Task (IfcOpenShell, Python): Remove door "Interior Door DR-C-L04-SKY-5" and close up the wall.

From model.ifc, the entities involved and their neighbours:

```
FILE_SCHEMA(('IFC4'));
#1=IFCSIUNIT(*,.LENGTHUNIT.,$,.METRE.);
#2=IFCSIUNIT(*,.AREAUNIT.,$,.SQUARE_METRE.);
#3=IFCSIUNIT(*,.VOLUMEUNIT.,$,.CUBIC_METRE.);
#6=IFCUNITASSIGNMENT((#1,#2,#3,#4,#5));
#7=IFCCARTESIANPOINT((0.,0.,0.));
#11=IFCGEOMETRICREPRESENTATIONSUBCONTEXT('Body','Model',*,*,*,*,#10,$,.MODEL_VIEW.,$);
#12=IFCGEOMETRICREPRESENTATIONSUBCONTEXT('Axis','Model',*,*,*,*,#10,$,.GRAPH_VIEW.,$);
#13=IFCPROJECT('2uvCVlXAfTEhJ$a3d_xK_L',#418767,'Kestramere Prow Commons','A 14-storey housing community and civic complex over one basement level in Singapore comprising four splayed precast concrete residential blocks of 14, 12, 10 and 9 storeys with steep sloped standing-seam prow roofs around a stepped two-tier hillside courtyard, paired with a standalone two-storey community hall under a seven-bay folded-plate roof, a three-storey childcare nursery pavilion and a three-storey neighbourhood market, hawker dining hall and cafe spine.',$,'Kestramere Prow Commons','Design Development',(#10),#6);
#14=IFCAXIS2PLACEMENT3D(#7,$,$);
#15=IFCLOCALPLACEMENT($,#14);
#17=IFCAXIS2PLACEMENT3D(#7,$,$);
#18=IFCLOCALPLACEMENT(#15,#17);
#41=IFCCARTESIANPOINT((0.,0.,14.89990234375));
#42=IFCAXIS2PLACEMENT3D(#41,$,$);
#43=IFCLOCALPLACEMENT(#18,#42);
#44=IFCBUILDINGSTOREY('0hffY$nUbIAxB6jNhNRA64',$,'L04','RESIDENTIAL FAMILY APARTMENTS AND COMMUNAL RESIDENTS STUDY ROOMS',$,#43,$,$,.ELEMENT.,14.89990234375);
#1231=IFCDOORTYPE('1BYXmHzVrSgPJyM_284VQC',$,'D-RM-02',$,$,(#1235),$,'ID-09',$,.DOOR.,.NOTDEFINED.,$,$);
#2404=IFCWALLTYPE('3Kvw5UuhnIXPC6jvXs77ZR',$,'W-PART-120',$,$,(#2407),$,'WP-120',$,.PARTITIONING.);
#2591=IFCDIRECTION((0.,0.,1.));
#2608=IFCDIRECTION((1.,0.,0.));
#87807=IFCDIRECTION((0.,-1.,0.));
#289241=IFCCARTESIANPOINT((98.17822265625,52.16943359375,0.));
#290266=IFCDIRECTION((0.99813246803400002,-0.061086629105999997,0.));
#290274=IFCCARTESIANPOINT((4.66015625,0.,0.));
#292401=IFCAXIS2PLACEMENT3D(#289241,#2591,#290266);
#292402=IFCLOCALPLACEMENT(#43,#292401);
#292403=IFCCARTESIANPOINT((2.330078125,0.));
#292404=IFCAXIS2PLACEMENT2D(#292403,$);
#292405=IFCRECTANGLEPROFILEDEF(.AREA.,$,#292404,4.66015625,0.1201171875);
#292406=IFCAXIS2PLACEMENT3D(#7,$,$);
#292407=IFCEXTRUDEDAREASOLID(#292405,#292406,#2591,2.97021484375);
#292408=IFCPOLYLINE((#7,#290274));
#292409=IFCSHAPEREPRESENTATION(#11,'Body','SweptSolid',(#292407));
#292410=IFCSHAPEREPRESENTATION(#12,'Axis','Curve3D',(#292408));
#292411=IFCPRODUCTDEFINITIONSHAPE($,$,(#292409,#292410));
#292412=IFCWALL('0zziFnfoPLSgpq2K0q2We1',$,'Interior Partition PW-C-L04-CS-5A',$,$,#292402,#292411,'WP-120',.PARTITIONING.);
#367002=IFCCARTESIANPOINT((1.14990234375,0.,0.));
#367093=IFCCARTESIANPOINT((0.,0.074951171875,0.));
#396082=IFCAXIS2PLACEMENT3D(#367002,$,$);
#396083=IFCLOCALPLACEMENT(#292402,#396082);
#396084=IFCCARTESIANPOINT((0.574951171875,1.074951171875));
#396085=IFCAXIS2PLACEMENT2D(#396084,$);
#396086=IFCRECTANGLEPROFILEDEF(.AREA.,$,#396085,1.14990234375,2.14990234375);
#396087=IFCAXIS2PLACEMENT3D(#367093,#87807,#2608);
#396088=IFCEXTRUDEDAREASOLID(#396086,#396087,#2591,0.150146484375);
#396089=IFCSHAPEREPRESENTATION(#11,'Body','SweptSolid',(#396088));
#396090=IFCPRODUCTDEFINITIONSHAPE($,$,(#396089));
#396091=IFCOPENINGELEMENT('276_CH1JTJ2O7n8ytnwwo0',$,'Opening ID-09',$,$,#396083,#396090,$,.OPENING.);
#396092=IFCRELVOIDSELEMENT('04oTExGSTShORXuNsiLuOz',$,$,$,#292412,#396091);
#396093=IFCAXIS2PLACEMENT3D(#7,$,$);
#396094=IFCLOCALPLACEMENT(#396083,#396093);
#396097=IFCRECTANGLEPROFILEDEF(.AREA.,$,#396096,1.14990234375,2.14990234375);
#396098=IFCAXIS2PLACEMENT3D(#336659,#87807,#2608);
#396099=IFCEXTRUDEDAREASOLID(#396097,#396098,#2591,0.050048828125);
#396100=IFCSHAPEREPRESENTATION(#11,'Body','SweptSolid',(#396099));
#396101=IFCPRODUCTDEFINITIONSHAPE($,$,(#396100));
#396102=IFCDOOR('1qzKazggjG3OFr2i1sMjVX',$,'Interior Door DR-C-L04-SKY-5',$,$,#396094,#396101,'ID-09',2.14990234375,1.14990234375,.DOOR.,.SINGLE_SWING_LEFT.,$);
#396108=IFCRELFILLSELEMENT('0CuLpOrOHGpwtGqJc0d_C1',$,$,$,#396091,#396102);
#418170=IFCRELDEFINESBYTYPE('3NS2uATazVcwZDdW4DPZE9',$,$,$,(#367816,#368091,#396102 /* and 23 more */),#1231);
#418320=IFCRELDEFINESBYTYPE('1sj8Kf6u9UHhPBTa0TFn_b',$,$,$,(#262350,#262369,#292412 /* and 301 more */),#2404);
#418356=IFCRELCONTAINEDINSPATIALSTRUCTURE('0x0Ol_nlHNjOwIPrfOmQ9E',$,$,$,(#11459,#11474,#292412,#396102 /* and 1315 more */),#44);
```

```python
import ifcopenshell
import ifcopenshell.api.feature
import ifcopenshell.api.root
import ifcopenshell.geom
import ifcopenshell.util.shape

model = ifcopenshell.open("model.ifc")
settings = ifcopenshell.geom.settings()


def volume(element):
    """Net volume in cubic metres, openings subtracted."""
    shape = ifcopenshell.geom.create_shape(settings, element)
    return ifcopenshell.util.shape.get_volume(shape.geometry)


door = model.by_guid("1qzKazggjG3OFr2i1sMjVX")
opening = door.FillsVoids[0].RelatingOpeningElement
wall = opening.VoidsElements[0].RelatingBuildingElement
before = volume(wall)

ifcopenshell.api.root.remove_product(model, product=door)
ifcopenshell.api.feature.remove_feature(model, feature=opening)

after = volume(wall)

print(f"wall volume {before:.3f} -> {after:.3f} m3")

model.write("model_updated.ifc")
```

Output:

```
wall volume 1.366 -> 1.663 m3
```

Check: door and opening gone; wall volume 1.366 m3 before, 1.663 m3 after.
